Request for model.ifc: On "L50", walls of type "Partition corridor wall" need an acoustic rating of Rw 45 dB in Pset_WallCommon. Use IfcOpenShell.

First a look at what the model holds.

```python
import ifcopenshell
import ifcopenshell.util.element

model = ifcopenshell.open("model.ifc")
print(model.schema)
storey = next(s for s in model.by_type("IfcBuildingStorey") if s.Name == "L50")
walls = [e for e in ifcopenshell.util.element.get_decomposition(storey) if e.is_a("IfcWall")]
seen = {}
for e in walls:
    element_type = ifcopenshell.util.element.get_type(e)
    key = (element_type.Name if element_type != e and element_type else None, ifcopenshell.util.element.get_pset(e, "Pset_WallCommon", "AcousticRating"))
    seen[key] = seen.get(key, 0) + 1
for (name, value), count in sorted(seen.items(), key=str):
    print(count, "x", name, "|", value)
```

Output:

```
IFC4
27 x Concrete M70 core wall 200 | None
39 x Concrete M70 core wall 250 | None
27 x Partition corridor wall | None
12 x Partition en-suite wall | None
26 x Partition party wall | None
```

```python
import ifcopenshell
import ifcopenshell.api.pset
import ifcopenshell.util.element

model = ifcopenshell.open("model.ifc")

storey = next(s for s in model.by_type("IfcBuildingStorey") if s.Name == "L50")
walls = [e for e in ifcopenshell.util.element.get_decomposition(storey) if e.is_a("IfcWall")]

count = 0
for e in walls:
    element_type = ifcopenshell.util.element.get_type(e)
    if element_type in (None, e) or element_type.Name != "Partition corridor wall":
        continue
    # add_pset returns the element's existing set when there is one.
    pset = ifcopenshell.api.pset.add_pset(model, product=e, name="Pset_WallCommon")
    ifcopenshell.api.pset.edit_pset(model, pset=pset, properties={"AcousticRating": "Rw 45 dB"})
    count += 1

print(count, "walls updated")

model.write("model_rev.ifc")
```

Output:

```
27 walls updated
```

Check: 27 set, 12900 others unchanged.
